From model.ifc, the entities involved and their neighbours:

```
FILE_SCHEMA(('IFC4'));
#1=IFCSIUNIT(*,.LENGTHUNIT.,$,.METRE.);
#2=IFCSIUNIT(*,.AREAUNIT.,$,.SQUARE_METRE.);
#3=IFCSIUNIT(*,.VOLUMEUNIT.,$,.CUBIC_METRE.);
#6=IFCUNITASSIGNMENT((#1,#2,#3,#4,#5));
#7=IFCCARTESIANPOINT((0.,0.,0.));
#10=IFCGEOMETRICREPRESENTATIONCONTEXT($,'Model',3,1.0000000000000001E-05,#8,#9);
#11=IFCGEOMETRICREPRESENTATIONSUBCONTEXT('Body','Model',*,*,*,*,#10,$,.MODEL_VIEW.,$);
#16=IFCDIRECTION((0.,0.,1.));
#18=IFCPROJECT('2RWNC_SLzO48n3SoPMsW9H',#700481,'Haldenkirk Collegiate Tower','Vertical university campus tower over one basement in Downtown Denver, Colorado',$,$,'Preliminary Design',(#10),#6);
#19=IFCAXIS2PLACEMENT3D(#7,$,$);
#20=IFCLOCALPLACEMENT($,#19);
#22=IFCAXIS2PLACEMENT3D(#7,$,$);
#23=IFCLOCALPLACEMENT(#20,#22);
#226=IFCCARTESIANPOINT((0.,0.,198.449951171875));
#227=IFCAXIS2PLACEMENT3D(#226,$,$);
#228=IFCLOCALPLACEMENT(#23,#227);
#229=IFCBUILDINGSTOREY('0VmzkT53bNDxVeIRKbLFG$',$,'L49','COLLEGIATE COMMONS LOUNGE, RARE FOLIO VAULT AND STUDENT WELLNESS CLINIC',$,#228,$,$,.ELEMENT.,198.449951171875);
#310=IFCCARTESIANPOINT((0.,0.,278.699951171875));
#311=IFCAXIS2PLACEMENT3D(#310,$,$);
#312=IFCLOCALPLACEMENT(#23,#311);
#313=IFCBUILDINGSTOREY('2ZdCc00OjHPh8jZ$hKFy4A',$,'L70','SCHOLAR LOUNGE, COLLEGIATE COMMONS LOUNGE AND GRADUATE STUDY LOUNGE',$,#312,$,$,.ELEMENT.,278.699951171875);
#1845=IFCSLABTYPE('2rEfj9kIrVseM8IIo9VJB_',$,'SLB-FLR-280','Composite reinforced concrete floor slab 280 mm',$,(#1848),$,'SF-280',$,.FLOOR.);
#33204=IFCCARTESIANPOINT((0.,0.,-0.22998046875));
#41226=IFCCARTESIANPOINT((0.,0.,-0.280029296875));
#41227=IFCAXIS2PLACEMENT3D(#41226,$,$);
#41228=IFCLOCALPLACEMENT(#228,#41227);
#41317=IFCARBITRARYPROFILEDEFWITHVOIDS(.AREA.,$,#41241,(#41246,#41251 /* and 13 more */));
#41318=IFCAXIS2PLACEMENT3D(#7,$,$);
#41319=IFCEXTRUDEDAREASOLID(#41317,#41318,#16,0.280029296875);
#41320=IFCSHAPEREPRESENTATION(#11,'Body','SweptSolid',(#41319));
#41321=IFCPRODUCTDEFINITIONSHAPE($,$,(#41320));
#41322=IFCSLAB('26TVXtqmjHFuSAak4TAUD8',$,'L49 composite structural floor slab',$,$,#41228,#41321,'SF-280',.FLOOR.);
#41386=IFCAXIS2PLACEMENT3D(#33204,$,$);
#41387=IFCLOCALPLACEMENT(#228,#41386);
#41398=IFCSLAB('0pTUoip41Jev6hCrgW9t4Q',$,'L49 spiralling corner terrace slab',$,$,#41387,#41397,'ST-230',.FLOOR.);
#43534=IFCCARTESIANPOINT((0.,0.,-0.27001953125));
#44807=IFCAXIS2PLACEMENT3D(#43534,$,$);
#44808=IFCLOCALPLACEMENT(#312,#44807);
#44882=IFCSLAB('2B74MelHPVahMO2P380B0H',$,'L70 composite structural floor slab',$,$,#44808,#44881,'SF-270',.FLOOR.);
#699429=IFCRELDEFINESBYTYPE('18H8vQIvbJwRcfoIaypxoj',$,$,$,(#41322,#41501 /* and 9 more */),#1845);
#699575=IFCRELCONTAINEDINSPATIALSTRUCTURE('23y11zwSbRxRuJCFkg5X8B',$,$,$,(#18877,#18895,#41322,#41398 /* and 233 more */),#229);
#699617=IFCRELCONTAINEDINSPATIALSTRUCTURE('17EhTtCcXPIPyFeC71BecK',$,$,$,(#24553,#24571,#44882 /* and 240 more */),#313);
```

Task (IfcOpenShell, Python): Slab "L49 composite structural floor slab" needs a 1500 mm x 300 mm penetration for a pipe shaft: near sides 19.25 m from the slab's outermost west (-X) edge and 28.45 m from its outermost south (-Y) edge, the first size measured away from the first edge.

```python
import numpy as np
import ifcopenshell
import ifcopenshell.api.feature
import ifcopenshell.api.geometry
import ifcopenshell.api.root
import ifcopenshell.geom
import ifcopenshell.util.placement
import ifcopenshell.util.representation
import ifcopenshell.util.shape
import ifcopenshell.util.unit

model = ifcopenshell.open("model.ifc")
unit_scale = ifcopenshell.util.unit.calculate_unit_scale(model)
settings = ifcopenshell.geom.settings()


def volume(element):
    """Net volume in cubic metres, openings subtracted."""
    shape = ifcopenshell.geom.create_shape(settings, element)
    return ifcopenshell.util.shape.get_volume(shape.geometry)


slab = model.by_guid("26TVXtqmjHFuSAak4TAUD8")
before = volume(slab)

# Extent in the slab's own axes, in metres. The edges named are its -X and -Y sides.
slab_shape = ifcopenshell.geom.create_shape(settings, slab)
vertices = ifcopenshell.util.shape.get_vertices(slab_shape.geometry)
x_min, y_min, bottom = vertices.min(axis=0)
top = vertices[:, 2].max()

opening = ifcopenshell.api.root.create_entity(model, ifc_class="IfcOpeningElement", name="Pipe shaft opening", predefined_type="OPENING")
context = ifcopenshell.util.representation.get_context(model, "Model", "Body", "MODEL_VIEW")
width, depth = 1.5, 0.3
outline = [(0.0, 0.0), (width, 0.0), (width, depth), (0.0, depth), (0.0, 0.0)]
# Overshoot both faces by 50 mm so the cut is clean.
shape = ifcopenshell.api.geometry.add_slab_representation(
    model, context=context, depth=top - bottom + 0.1, polyline=outline
)
ifcopenshell.api.geometry.assign_representation(model, product=opening, representation=shape)

matrix = ifcopenshell.util.placement.get_local_placement(slab.ObjectPlacement)
matrix[:, 3] = matrix @ np.append(np.array([x_min + 19.25, y_min + 28.45, bottom - 0.05]) / unit_scale, 1.0)
ifcopenshell.api.geometry.edit_object_placement(model, product=opening, matrix=matrix, is_si=False)
ifcopenshell.api.feature.add_feature(model, feature=opening, element=slab)

after = volume(slab)

print(f"slab volume {before:.3f} -> {after:.3f} m3")

model.write("model_v2.ifc")
```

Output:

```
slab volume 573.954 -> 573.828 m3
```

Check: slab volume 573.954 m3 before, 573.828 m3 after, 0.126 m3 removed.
